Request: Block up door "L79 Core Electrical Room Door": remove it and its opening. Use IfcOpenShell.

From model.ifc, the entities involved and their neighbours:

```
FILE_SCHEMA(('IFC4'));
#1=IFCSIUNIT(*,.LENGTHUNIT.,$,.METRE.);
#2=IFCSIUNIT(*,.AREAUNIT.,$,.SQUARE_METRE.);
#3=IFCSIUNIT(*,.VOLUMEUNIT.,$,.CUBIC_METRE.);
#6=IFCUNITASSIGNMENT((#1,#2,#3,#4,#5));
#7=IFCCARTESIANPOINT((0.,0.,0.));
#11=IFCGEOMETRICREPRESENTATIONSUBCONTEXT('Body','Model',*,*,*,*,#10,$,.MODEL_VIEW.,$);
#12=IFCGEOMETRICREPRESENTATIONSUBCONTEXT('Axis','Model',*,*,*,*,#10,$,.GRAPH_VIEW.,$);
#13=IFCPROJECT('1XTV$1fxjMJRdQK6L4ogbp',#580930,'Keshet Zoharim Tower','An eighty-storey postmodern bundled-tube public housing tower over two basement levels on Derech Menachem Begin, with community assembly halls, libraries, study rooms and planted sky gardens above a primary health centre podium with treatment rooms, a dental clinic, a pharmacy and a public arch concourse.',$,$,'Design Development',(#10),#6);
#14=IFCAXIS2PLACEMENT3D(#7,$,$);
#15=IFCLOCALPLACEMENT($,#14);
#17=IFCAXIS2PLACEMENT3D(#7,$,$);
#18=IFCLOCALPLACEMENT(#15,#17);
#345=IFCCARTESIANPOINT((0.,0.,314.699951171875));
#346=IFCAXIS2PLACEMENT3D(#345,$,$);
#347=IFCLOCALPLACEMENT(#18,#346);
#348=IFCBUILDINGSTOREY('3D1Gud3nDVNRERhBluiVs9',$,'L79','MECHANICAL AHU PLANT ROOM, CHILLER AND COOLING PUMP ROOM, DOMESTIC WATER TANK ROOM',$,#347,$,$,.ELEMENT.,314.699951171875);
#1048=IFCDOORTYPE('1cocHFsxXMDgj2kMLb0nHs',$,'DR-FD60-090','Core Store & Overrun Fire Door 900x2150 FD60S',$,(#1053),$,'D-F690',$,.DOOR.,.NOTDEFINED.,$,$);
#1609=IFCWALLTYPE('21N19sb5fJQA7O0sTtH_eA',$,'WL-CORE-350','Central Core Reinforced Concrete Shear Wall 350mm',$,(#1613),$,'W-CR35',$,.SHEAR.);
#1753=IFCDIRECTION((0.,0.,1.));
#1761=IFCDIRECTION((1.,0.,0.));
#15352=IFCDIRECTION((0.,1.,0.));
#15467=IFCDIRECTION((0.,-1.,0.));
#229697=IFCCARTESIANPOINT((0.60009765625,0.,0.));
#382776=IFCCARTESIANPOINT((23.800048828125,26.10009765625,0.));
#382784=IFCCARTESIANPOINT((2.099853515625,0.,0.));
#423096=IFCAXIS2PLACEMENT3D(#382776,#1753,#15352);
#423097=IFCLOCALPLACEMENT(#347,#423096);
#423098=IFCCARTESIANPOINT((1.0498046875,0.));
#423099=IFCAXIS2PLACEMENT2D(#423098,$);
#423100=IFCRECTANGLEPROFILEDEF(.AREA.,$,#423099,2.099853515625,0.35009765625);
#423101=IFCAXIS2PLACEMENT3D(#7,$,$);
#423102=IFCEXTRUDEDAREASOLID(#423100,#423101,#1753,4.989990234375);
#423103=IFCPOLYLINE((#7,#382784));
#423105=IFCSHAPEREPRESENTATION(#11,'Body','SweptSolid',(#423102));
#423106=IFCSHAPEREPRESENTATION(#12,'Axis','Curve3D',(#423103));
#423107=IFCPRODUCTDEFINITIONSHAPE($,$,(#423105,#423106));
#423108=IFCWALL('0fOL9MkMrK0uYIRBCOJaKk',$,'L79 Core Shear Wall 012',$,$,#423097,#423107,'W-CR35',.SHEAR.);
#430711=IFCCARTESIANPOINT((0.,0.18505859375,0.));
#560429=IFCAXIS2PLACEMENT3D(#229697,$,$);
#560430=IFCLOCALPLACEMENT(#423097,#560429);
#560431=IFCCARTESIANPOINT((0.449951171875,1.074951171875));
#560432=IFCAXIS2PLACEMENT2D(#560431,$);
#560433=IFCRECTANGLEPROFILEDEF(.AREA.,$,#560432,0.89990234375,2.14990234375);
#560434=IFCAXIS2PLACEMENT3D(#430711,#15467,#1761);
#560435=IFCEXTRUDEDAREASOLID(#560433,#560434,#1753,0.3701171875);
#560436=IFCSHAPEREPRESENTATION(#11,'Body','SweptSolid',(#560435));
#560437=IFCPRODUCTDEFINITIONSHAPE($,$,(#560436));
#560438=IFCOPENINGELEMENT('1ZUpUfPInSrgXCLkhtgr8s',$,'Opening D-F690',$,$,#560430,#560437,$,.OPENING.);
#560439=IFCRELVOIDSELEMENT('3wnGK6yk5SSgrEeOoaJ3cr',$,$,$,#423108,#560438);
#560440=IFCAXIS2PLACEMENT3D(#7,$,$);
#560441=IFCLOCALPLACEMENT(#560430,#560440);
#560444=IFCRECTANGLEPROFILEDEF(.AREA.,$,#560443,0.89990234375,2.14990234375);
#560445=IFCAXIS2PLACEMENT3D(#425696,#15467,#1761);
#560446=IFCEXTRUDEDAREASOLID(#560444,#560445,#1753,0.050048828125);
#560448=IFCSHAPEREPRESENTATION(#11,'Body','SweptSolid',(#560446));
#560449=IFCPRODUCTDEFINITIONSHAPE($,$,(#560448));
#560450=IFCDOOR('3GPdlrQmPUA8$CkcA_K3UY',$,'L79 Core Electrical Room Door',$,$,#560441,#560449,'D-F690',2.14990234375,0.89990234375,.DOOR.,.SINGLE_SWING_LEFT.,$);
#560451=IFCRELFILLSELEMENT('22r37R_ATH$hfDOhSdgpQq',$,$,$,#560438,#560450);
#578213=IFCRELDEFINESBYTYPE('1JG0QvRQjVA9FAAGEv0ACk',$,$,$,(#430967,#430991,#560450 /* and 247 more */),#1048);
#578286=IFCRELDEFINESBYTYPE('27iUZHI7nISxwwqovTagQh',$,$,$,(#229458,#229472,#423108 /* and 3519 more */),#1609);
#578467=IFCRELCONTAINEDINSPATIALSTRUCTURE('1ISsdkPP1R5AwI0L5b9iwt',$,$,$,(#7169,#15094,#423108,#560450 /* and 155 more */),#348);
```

```python
import ifcopenshell
import ifcopenshell.api.feature
import ifcopenshell.api.root
import ifcopenshell.geom
import ifcopenshell.util.shape

model = ifcopenshell.open("model.ifc")
settings = ifcopenshell.geom.settings()


def volume(element):
    """Net volume in cubic metres, openings subtracted."""
    shape = ifcopenshell.geom.create_shape(settings, element)
    return ifcopenshell.util.shape.get_volume(shape.geometry)


door = model.by_guid("3GPdlrQmPUA8$CkcA_K3UY")
opening = door.FillsVoids[0].RelatingOpeningElement
wall = opening.VoidsElements[0].RelatingBuildingElement
before = volume(wall)

ifcopenshell.api.root.remove_product(model, product=door)
ifcopenshell.api.feature.remove_feature(model, feature=opening)

after = volume(wall)

print(f"wall volume {before:.3f} -> {after:.3f} m3")

model.write("model_rev.ifc")
```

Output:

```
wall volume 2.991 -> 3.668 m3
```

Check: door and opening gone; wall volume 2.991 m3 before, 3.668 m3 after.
